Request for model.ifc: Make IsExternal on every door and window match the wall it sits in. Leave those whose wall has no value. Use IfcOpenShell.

First a look at what the model holds.

```python
import ifcopenshell
import ifcopenshell.util.element

model = ifcopenshell.open("model.ifc")
print(model.schema)
seen = {}
for e in model.by_type("IfcDoor") + model.by_type("IfcWindow"):
    if not e.FillsVoids:
        continue
    host = e.FillsVoids[0].RelatingOpeningElement.VoidsElements[0].RelatingBuildingElement
    own = ifcopenshell.util.element.get_pset(e, f"Pset_{e.is_a()[3:].removesuffix('StandardCase')}Common", "IsExternal")
    wall = ifcopenshell.util.element.get_pset(host, "Pset_WallCommon", "IsExternal")
    seen[e.is_a(), own, wall] = seen.get((e.is_a(), own, wall), 0) + 1
for (cls, own, wall), count in sorted(seen.items(), key=str):
    print(count, cls, "IsExternal:", own, "| host wall:", wall)
```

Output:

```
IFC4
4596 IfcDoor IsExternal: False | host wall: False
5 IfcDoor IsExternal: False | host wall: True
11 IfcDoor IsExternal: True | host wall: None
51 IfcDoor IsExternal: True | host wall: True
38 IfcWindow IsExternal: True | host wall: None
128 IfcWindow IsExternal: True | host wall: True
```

```python
import ifcopenshell
import ifcopenshell.api.pset
import ifcopenshell.util.element

model = ifcopenshell.open("model.ifc")

count = 0
for ifc_class, pset_name in (("IfcDoor", "Pset_DoorCommon"), ("IfcWindow", "Pset_WindowCommon")):
    for e in model.by_type(ifc_class):
        if not e.FillsVoids:
            continue
        host = e.FillsVoids[0].RelatingOpeningElement.VoidsElements[0].RelatingBuildingElement
        external = ifcopenshell.util.element.get_pset(host, "Pset_WallCommon", "IsExternal")
        if external is None or ifcopenshell.util.element.get_pset(e, pset_name, "IsExternal") == external:
            continue
        pset = ifcopenshell.api.pset.add_pset(model, product=e, name=pset_name)
        ifcopenshell.api.pset.edit_pset(model, pset=pset, properties={"IsExternal": external})
        count += 1

print(count, "updated")

model.write("model_rev.ifc")
```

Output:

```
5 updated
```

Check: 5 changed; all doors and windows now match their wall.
